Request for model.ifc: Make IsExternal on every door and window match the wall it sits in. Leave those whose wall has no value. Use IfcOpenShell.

First a look at what the model holds.

```python
import ifcopenshell
import ifcopenshell.util.element

model = ifcopenshell.open("model.ifc")
print(model.schema)
seen = {}
for e in model.by_type("IfcDoor") + model.by_type("IfcWindow"):
    if not e.FillsVoids:
        continue
    host = e.FillsVoids[0].RelatingOpeningElement.VoidsElements[0].RelatingBuildingElement
    own = ifcopenshell.util.element.get_pset(e, f"Pset_{e.is_a()[3:].removesuffix('StandardCase')}Common", "IsExternal")
    wall = ifcopenshell.util.element.get_pset(host, "Pset_WallCommon", "IsExternal")
    seen[e.is_a(), own, wall] = seen.get((e.is_a(), own, wall), 0) + 1
for (cls, own, wall), count in sorted(seen.items(), key=str):
    print(count, cls, "IsExternal:", own, "| host wall:", wall)
```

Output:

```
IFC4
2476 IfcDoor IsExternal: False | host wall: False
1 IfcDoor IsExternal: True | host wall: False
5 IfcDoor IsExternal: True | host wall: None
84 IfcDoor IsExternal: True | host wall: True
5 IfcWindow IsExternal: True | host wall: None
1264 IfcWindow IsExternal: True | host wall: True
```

```python
import ifcopenshell
import ifcopenshell.api.pset
import ifcopenshell.util.element

model = ifcopenshell.open("model.ifc")

count = 0
for ifc_class, pset_name in (("IfcDoor", "Pset_DoorCommon"), ("IfcWindow", "Pset_WindowCommon")):
    for e in model.by_type(ifc_class):
        if not e.FillsVoids:
            continue
        host = e.FillsVoids[0].RelatingOpeningElement.VoidsElements[0].RelatingBuildingElement
        external = ifcopenshell.util.element.get_pset(host, "Pset_WallCommon", "IsExternal")
        if external is None or ifcopenshell.util.element.get_pset(e, pset_name, "IsExternal") == external:
            continue
        pset = ifcopenshell.api.pset.add_pset(model, product=e, name=pset_name)
        ifcopenshell.api.pset.edit_pset(model, pset=pset, properties={"IsExternal": external})
        count += 1

print(count, "updated")

model.write("model_v2.ifc")
```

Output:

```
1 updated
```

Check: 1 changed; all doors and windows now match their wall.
